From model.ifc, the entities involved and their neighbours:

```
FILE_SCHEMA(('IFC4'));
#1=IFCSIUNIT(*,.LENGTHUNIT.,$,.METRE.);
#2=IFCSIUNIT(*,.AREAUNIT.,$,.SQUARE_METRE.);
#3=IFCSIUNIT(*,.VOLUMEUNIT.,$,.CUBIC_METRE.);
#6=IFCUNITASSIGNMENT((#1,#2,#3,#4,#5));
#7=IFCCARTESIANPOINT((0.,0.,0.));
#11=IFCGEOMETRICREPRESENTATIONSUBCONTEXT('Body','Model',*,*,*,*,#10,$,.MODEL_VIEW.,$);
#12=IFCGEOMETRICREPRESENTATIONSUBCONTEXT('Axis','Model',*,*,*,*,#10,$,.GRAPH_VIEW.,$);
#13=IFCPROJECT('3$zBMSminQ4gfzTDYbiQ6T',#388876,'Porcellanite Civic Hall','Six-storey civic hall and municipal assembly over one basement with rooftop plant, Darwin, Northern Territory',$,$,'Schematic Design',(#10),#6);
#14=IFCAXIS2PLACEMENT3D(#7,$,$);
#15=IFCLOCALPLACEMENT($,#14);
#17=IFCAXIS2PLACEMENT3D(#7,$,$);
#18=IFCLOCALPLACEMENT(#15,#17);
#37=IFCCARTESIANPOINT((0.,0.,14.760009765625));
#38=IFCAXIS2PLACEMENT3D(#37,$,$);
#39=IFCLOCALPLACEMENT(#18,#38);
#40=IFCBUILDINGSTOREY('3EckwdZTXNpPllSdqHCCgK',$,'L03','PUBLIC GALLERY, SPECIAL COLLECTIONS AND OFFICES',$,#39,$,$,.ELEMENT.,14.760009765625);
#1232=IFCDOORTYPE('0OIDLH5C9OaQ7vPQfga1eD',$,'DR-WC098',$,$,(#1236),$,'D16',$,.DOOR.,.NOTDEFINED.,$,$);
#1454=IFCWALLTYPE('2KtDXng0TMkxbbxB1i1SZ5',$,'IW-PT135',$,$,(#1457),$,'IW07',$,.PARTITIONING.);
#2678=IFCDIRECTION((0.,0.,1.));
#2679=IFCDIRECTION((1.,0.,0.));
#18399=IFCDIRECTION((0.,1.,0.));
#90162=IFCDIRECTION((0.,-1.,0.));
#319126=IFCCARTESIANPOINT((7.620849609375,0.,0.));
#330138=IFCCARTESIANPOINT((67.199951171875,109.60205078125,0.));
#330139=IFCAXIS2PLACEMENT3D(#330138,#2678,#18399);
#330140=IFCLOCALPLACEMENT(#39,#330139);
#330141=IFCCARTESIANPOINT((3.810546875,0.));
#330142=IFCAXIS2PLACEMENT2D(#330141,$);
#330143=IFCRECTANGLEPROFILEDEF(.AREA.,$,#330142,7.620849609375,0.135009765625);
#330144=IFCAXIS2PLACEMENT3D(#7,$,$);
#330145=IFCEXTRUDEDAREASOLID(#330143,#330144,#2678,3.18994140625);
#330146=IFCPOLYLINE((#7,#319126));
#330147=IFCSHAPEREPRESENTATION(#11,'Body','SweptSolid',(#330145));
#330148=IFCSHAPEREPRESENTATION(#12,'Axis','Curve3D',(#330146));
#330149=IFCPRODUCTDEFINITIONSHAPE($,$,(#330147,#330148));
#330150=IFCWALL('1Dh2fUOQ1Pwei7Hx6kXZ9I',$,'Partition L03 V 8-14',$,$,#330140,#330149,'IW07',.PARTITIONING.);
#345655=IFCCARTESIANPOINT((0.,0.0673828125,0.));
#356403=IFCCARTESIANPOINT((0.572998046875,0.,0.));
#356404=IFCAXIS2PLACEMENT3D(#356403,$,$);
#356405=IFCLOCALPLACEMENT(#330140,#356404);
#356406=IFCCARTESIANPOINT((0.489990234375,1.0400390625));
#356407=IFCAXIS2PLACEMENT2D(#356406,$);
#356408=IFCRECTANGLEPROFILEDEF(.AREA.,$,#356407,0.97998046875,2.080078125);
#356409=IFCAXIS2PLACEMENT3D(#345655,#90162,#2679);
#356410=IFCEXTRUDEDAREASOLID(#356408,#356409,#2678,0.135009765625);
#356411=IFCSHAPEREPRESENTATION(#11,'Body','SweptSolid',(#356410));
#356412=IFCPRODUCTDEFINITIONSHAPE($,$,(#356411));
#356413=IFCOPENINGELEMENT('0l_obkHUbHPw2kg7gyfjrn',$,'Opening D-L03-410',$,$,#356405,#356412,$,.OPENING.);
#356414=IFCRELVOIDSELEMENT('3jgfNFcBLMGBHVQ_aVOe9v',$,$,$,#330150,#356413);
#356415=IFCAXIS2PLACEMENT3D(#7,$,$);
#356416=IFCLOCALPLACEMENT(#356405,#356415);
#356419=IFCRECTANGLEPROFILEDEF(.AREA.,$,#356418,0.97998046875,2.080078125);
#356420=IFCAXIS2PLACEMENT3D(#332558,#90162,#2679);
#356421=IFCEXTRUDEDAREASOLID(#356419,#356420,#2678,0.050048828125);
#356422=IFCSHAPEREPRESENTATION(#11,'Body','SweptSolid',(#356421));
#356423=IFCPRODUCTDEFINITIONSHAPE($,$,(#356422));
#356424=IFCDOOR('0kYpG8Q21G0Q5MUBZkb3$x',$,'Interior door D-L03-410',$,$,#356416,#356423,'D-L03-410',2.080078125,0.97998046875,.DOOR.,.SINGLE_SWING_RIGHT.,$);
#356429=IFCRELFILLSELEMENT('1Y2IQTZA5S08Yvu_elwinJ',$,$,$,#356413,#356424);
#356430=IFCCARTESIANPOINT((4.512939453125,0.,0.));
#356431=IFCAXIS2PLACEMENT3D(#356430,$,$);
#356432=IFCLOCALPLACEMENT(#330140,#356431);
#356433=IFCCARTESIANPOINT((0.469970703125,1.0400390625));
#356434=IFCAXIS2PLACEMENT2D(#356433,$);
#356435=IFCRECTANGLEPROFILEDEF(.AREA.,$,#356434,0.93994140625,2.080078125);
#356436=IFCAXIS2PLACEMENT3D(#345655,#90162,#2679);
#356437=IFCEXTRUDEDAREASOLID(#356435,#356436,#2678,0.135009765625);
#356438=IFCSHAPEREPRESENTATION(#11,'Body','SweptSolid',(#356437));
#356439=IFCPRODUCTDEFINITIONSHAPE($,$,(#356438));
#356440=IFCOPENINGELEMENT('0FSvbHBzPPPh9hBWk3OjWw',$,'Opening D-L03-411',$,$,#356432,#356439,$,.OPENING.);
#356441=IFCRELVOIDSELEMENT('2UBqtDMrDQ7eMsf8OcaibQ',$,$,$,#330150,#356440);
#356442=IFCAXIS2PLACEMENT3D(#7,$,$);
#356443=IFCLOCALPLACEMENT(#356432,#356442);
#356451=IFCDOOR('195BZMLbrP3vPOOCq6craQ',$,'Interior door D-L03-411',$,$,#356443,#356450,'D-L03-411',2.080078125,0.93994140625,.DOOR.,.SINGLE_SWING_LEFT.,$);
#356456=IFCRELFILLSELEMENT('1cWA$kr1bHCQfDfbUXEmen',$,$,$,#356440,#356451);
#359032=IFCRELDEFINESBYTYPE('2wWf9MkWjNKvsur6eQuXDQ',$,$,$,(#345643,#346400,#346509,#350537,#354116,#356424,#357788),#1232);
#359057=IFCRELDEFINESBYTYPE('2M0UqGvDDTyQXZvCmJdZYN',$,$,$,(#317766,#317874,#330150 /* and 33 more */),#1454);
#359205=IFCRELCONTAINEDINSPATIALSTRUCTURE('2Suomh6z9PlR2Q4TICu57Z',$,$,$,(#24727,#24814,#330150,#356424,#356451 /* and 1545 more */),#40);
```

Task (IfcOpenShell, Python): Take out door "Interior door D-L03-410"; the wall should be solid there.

```python
import ifcopenshell
import ifcopenshell.api.feature
import ifcopenshell.api.root
import ifcopenshell.geom
import ifcopenshell.util.shape

model = ifcopenshell.open("model.ifc")
settings = ifcopenshell.geom.settings()


def volume(element):
    """Net volume in cubic metres, openings subtracted."""
    shape = ifcopenshell.geom.create_shape(settings, element)
    return ifcopenshell.util.shape.get_volume(shape.geometry)


door = model.by_guid("0kYpG8Q21G0Q5MUBZkb3$x")
opening = door.FillsVoids[0].RelatingOpeningElement
wall = opening.VoidsElements[0].RelatingBuildingElement
before = volume(wall)

ifcopenshell.api.root.remove_product(model, product=door)
ifcopenshell.api.feature.remove_feature(model, feature=opening)

after = volume(wall)

print(f"wall volume {before:.3f} -> {after:.3f} m3")

model.write("model_v2.ifc")
```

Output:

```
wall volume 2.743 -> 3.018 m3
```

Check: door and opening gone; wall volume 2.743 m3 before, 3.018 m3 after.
